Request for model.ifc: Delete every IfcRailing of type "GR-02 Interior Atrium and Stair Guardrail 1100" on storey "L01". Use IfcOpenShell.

First a look at what the model holds.

```python
import ifcopenshell
import ifcopenshell.util.element

model = ifcopenshell.open("model.ifc")
print(model.schema)
storey = next(s for s in model.by_type("IfcBuildingStorey") if s.Name == "L01")
railings = [e for e in ifcopenshell.util.element.get_decomposition(storey) if e.is_a("IfcRailing")]
seen = {}
for e in railings:
    element_type = ifcopenshell.util.element.get_type(e)
    name = element_type.Name if element_type not in (None, e) else None
    seen[name] = seen.get(name, 0) + 1
for name, count in sorted(seen.items(), key=str):
    print(count, "x", name)
```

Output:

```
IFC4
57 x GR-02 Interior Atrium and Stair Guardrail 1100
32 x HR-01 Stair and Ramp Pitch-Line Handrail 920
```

```python
import ifcopenshell
import ifcopenshell.api.root
import ifcopenshell.util.element

model = ifcopenshell.open("model.ifc")

storey = next(s for s in model.by_type("IfcBuildingStorey") if s.Name == "L01")
railings = [e for e in ifcopenshell.util.element.get_decomposition(storey) if e.is_a("IfcRailing")]
targets = [e for e in railings if (t := ifcopenshell.util.element.get_type(e)) not in (None, e) and t.Name == "GR-02 Interior Atrium and Stair Guardrail 1100"]

for e in targets:
    ifcopenshell.api.root.remove_product(model, product=e)
print(len(targets), "removed")

model.write("model_v2.ifc")
```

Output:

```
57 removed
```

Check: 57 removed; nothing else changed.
